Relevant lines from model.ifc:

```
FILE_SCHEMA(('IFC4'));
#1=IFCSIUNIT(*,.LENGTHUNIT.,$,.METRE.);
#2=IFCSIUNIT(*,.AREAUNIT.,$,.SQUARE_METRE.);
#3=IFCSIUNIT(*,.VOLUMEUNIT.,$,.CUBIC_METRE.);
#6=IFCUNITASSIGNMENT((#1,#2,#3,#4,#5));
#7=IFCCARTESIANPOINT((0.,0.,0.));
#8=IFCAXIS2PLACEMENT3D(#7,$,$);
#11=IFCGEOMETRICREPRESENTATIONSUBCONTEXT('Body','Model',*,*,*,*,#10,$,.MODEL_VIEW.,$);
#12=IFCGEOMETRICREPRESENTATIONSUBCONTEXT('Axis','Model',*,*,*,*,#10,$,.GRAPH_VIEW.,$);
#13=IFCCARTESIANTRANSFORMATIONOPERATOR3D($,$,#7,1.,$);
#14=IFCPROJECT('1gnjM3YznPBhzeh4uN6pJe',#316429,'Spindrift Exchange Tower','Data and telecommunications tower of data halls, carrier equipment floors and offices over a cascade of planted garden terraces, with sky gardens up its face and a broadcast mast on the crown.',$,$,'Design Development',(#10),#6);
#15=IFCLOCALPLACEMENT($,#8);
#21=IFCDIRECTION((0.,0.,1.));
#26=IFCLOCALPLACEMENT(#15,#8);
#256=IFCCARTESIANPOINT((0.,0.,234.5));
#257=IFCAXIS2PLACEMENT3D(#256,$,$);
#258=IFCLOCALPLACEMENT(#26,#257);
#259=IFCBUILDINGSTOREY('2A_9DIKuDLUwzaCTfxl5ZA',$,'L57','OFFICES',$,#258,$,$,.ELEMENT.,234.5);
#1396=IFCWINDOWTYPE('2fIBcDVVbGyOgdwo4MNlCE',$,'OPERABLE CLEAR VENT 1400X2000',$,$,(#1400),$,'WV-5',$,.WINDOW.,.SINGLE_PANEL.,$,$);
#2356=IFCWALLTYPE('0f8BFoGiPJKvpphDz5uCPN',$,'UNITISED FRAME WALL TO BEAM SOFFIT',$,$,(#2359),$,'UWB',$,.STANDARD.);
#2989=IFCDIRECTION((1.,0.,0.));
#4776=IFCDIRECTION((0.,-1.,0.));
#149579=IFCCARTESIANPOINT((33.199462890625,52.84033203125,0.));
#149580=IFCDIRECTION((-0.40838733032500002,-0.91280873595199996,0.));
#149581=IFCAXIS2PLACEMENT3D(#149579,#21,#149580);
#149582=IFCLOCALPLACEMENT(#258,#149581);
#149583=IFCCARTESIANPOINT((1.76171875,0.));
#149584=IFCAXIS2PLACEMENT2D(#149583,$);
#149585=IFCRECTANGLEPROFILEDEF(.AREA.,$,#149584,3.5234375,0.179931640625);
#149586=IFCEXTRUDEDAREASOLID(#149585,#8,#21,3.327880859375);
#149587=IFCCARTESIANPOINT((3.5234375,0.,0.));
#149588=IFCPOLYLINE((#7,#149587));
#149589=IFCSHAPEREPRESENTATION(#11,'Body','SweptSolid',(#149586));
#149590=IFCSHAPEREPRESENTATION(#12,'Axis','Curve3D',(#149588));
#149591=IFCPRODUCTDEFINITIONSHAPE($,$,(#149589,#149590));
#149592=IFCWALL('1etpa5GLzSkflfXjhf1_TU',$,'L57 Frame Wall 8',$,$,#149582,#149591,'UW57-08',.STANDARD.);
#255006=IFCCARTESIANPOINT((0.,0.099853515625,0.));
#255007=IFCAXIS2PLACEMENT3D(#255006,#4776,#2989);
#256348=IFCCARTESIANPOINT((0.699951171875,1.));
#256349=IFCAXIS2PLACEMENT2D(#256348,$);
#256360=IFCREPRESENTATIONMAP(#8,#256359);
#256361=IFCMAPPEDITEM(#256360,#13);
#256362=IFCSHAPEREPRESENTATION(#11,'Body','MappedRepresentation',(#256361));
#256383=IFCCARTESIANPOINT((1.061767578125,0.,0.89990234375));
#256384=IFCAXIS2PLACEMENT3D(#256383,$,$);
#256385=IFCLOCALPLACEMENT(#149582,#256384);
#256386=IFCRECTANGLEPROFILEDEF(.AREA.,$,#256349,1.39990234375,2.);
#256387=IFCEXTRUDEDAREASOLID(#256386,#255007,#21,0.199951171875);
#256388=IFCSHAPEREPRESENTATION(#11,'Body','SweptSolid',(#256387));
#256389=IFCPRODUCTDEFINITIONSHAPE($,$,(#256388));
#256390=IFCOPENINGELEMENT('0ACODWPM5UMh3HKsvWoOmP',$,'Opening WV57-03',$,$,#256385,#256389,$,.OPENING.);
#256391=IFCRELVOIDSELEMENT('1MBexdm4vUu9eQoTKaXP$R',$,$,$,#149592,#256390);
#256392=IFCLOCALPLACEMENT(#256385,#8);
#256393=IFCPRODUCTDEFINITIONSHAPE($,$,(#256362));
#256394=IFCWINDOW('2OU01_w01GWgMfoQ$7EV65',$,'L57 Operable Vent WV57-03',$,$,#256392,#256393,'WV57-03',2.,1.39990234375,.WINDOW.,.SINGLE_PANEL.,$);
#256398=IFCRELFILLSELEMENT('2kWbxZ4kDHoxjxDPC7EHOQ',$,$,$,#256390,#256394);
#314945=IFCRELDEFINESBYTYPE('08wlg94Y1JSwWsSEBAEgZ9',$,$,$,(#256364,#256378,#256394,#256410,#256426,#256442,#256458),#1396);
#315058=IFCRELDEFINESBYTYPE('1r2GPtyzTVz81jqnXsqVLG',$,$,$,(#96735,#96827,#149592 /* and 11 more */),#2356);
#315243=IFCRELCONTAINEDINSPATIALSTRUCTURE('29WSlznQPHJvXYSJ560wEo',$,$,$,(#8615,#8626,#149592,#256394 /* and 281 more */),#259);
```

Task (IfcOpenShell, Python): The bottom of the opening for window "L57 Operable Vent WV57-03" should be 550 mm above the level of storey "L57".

```python
import numpy as np
import ifcopenshell
import ifcopenshell.api.geometry
import ifcopenshell.geom
import ifcopenshell.util.element
import ifcopenshell.util.placement
import ifcopenshell.util.shape
import ifcopenshell.util.unit

model = ifcopenshell.open("model.ifc")
unit_scale = ifcopenshell.util.unit.calculate_unit_scale(model)

window = model.by_guid("2OU01_w01GWgMfoQ$7EV65")
opening = window.FillsVoids[0].RelatingOpeningElement
storey = ifcopenshell.util.element.get_container(window, ifc_class="IfcBuildingStorey")
level = ifcopenshell.util.placement.get_local_placement(storey.ObjectPlacement)[2, 3]

# The opening's origin need not be at the sill, so measure its lowest point.
shape = ifcopenshell.geom.create_shape(ifcopenshell.geom.settings(), opening)
bottom = ifcopenshell.util.shape.get_shape_bottom_elevation(shape, shape.geometry) / unit_scale
dz = level + 0.55 / unit_scale - bottom

shift = np.array([0.0, 0.0, dz])
# The window is placed relative to its opening, so it follows when the opening moves.
matrix = ifcopenshell.util.placement.get_local_placement(opening.ObjectPlacement)
matrix[:3, 3] += shift
ifcopenshell.api.geometry.edit_object_placement(
    model, product=opening, matrix=matrix, is_si=False, should_transform_children=True
)

print(f"moved by {dz * unit_scale:+.3f} m")

model.write("model_rev.ifc")
```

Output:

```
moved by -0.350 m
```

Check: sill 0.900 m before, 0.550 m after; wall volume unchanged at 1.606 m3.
